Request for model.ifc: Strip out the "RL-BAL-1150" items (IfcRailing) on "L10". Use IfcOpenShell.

First a look at what the model holds.

```python
import ifcopenshell
import ifcopenshell.util.element

model = ifcopenshell.open("model.ifc")
print(model.schema)
storey = next(s for s in model.by_type("IfcBuildingStorey") if s.Name == "L10")
railings = [e for e in ifcopenshell.util.element.get_decomposition(storey) if e.is_a("IfcRailing")]
seen = {}
for e in railings:
    element_type = ifcopenshell.util.element.get_type(e)
    name = element_type.Name if element_type not in (None, e) else None
    seen[name] = seen.get(name, 0) + 1
for name, count in sorted(seen.items(), key=str):
    print(count, "x", name)
```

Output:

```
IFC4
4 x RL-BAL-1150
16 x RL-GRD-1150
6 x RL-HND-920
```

```python
import ifcopenshell
import ifcopenshell.api.root
import ifcopenshell.util.element

model = ifcopenshell.open("model.ifc")

storey = next(s for s in model.by_type("IfcBuildingStorey") if s.Name == "L10")
railings = [e for e in ifcopenshell.util.element.get_decomposition(storey) if e.is_a("IfcRailing")]
targets = [e for e in railings if (t := ifcopenshell.util.element.get_type(e)) not in (None, e) and t.Name == "RL-BAL-1150"]

for e in targets:
    ifcopenshell.api.root.remove_product(model, product=e)
print(len(targets), "removed")

model.write("model_edited.ifc")
```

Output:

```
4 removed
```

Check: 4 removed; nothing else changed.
